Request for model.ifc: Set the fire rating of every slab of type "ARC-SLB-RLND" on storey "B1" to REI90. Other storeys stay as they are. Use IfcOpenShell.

First a look at what the model holds.

```python
import ifcopenshell
import ifcopenshell.util.element

model = ifcopenshell.open("model.ifc")
print(model.schema)
storey = next(s for s in model.by_type("IfcBuildingStorey") if s.Name == "B1")
slabs = [e for e in ifcopenshell.util.element.get_decomposition(storey) if e.is_a("IfcSlab")]
seen = {}
for e in slabs:
    element_type = ifcopenshell.util.element.get_type(e)
    key = (element_type.Name if element_type != e and element_type else None, ifcopenshell.util.element.get_pset(e, "Pset_SlabCommon", "FireRating"))
    seen[key] = seen.get(key, 0) + 1
for (name, value), count in sorted(seen.items(), key=str):
    print(count, "x", name, "|", value)
```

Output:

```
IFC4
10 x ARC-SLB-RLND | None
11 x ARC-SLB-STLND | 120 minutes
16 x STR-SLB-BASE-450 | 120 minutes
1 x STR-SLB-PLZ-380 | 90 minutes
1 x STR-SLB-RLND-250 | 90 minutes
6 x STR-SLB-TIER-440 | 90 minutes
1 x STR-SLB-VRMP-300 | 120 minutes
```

```python
import ifcopenshell
import ifcopenshell.api.pset
import ifcopenshell.util.element

model = ifcopenshell.open("model.ifc")

storey = next(s for s in model.by_type("IfcBuildingStorey") if s.Name == "B1")
slabs = [e for e in ifcopenshell.util.element.get_decomposition(storey) if e.is_a("IfcSlab")]

count = 0
for e in slabs:
    element_type = ifcopenshell.util.element.get_type(e)
    if element_type in (None, e) or element_type.Name != "ARC-SLB-RLND":
        continue
    # add_pset returns the element's existing set when there is one.
    pset = ifcopenshell.api.pset.add_pset(model, product=e, name="Pset_SlabCommon")
    ifcopenshell.api.pset.edit_pset(model, pset=pset, properties={"FireRating": "REI90"})
    count += 1

print(count, "slabs updated")

model.write("model_updated.ifc")
```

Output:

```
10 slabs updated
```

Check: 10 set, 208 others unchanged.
